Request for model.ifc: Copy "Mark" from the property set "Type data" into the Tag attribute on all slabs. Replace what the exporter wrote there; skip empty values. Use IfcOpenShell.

First a look at what the model holds.

```python
import ifcopenshell
import ifcopenshell.util.element

model = ifcopenshell.open("model.ifc")
print(model.schema)
slabs = model.by_type("IfcSlab")
print(len(slabs), "slabs")
for e in slabs[:8]:
    source = ifcopenshell.util.element.get_pset(e, "Type data", "Mark")
    target = e.Tag
    print(e.id(), repr(source), repr(target), sep=" | ")
```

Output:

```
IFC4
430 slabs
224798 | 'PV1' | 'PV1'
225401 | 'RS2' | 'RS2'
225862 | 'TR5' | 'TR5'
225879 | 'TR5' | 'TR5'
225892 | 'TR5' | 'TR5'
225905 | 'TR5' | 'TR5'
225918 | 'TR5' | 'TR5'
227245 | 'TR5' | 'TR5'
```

```python
import ifcopenshell
import ifcopenshell.util.element

model = ifcopenshell.open("model.ifc")

count = 0
for e in model.by_type("IfcSlab"):
    value = ifcopenshell.util.element.get_pset(e, "Type data", "Mark")
    current = e.Tag
    if not value or not value.strip() or current == value:
        continue
    e.Tag = value
    count += 1

print(count, "slabs updated")

model.write("model_edited.ifc")
```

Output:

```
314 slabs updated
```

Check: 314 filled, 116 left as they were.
